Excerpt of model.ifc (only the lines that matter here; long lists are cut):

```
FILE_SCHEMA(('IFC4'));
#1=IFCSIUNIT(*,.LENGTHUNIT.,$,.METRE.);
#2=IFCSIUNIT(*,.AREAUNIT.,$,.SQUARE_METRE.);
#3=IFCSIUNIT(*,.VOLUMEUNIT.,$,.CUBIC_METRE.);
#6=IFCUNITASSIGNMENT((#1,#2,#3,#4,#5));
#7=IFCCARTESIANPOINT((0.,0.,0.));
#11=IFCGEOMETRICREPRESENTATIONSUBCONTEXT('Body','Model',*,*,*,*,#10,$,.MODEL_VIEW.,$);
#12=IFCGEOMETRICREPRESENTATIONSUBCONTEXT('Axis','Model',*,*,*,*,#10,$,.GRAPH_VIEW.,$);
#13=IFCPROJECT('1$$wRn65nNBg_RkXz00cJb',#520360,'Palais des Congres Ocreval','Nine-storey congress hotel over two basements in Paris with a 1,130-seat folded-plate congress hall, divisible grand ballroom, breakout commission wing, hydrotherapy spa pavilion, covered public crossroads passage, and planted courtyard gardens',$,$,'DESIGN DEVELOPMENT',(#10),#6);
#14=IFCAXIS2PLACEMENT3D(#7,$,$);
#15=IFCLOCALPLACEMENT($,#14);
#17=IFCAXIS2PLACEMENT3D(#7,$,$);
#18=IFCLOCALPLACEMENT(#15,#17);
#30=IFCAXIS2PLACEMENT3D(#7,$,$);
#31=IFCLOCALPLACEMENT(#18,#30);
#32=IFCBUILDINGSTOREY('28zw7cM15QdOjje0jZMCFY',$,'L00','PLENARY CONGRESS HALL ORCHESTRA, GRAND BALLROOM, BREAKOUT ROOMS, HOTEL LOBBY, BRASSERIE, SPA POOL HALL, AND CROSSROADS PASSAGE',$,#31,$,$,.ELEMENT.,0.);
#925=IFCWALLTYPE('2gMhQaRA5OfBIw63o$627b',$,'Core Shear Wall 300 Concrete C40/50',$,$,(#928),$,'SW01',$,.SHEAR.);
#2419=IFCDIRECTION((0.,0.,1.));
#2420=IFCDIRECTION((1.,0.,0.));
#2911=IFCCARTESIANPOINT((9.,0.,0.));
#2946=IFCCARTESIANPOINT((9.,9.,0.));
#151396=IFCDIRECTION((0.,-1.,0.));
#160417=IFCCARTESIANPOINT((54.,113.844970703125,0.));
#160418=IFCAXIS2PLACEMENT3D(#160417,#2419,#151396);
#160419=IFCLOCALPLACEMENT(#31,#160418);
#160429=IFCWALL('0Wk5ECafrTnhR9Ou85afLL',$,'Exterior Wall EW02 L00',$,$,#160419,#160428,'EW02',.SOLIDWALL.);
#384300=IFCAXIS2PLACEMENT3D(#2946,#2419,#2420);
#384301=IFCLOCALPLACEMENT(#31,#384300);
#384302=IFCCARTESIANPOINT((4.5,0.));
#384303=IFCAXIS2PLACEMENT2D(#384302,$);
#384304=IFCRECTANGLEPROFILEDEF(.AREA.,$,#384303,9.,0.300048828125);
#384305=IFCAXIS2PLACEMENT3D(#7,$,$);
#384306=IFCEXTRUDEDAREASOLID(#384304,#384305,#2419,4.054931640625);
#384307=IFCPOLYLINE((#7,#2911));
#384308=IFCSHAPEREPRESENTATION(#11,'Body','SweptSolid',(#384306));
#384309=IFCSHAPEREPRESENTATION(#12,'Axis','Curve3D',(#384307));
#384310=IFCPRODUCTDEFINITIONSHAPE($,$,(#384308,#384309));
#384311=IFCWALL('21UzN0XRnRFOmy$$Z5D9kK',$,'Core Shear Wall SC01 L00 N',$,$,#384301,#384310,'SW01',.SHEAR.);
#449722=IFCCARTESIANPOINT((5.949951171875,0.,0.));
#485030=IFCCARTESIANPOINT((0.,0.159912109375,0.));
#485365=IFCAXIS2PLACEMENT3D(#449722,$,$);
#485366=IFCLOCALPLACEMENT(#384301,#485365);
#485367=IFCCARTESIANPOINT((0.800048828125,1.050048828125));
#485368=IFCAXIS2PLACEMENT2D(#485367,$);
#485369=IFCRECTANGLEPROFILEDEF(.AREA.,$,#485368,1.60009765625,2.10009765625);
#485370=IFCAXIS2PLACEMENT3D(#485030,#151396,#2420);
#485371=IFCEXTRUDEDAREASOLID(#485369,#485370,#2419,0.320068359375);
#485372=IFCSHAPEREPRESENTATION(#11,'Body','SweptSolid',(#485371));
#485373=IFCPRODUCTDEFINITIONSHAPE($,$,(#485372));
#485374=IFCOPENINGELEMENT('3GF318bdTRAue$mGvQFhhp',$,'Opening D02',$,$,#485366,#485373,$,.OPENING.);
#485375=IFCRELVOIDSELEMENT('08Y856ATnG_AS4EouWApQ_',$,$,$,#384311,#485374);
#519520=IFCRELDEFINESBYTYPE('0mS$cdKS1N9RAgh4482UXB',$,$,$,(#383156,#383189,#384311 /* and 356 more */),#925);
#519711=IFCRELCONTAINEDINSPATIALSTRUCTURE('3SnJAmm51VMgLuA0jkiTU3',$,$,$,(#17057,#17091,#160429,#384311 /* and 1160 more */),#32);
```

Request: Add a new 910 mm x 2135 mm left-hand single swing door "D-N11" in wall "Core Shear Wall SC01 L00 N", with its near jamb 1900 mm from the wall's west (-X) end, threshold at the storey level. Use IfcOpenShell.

```python
import numpy as np
import ifcopenshell
import ifcopenshell.api.feature
import ifcopenshell.api.geometry
import ifcopenshell.api.root
import ifcopenshell.api.spatial
import ifcopenshell.geom
import ifcopenshell.util.element
import ifcopenshell.util.placement
import ifcopenshell.util.representation
import ifcopenshell.util.shape
import ifcopenshell.util.unit

model = ifcopenshell.open("model.ifc")
unit_scale = ifcopenshell.util.unit.calculate_unit_scale(model)
settings = ifcopenshell.geom.settings()


def volume(element):
    """Net volume in cubic metres, openings subtracted."""
    shape = ifcopenshell.geom.create_shape(settings, element)
    return ifcopenshell.util.shape.get_volume(shape.geometry)


wall = model.by_guid("21UzN0XRnRFOmy$$Z5D9kK")
storey = ifcopenshell.util.element.get_container(wall, ifc_class="IfcBuildingStorey")
context = ifcopenshell.util.representation.get_context(model, "Model", "Body", "MODEL_VIEW")
before = volume(wall)

width, height, from_end, sill = 0.91, 2.135, 1.9, 0.0  # metres

# The wall runs along its own X axis, and the end named is its -X end.
wall_shape = ifcopenshell.geom.create_shape(settings, wall)
x, y, z = ifcopenshell.util.shape.get_vertices(wall_shape.geometry).T
start = x.min() + from_end
face, thickness = float(y.min()), float(y.max() - y.min())
wall_matrix = ifcopenshell.util.placement.get_local_placement(wall.ObjectPlacement)
level = ifcopenshell.util.placement.get_local_placement(storey.ObjectPlacement)[2, 3]


def in_wall(x, y):
    """Placement at x, y metres in the wall's axes, at sill height."""
    matrix = wall_matrix.copy()
    matrix[:, 3] = wall_matrix @ np.array([x / unit_scale, y / unit_scale, 0.0, 1.0])
    matrix[2, 3] = level + sill / unit_scale
    return matrix


# Opening: a box that overshoots both wall faces by 50 mm.
opening = ifcopenshell.api.root.create_entity(model, ifc_class="IfcOpeningElement", predefined_type="OPENING")
box = ifcopenshell.api.geometry.add_wall_representation(
    model, context=context, length=width, height=height, thickness=thickness + 0.1
)
ifcopenshell.api.geometry.assign_representation(model, product=opening, representation=box)
ifcopenshell.api.geometry.edit_object_placement(model, product=opening, matrix=in_wall(start, face - 0.05), is_si=False)
ifcopenshell.api.feature.add_feature(model, feature=opening, element=wall)

door = ifcopenshell.api.root.create_entity(model, ifc_class="IfcDoor", name="D-N11", predefined_type="DOOR")
door.OverallWidth, door.OverallHeight = width / unit_scale, height / unit_scale
door.OperationType = "SINGLE_SWING_LEFT"
body = ifcopenshell.api.geometry.add_door_representation(
    model,
    context=context,
    overall_width=door.OverallWidth,
    overall_height=door.OverallHeight,
    operation_type="SINGLE_SWING_LEFT",
    lining_properties={"LiningDepth": thickness / unit_scale, "ThresholdDepth": thickness / unit_scale},
)
ifcopenshell.api.geometry.assign_representation(model, product=door, representation=body)
ifcopenshell.api.spatial.assign_container(model, products=[door], relating_structure=storey)
ifcopenshell.api.feature.add_filling(model, opening=opening, element=door)

# The lining spans the wall, so the door starts at the wall face.
ifcopenshell.api.geometry.edit_object_placement(model, product=door, matrix=in_wall(start, face), is_si=False)

after = volume(wall)

print(f"wall volume {before:.3f} -> {after:.3f} m3")

model.write("model_edited.ifc")
```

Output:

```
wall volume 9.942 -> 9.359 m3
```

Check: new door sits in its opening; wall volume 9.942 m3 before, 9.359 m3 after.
